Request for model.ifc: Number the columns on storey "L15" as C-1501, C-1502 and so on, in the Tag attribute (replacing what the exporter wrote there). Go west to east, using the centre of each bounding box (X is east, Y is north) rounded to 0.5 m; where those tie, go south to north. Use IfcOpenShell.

First a look at what the model holds.

```python
import ifcopenshell
import ifcopenshell.util.element
import ifcopenshell.util.placement

model = ifcopenshell.open("model.ifc")
print(model.schema)
storey = next(s for s in model.by_type("IfcBuildingStorey") if s.Name == "L15")
columns = [e for e in ifcopenshell.util.element.get_decomposition(storey) if e.is_a("IfcColumn")]
for e in sorted(columns, key=lambda e: e.id()):
    origin = ifcopenshell.util.placement.get_local_placement(e.ObjectPlacement)[:3, 3]
    print(e.id(), e.Tag, e.Name, origin.round(2) + 0.0, sep=" | ")
```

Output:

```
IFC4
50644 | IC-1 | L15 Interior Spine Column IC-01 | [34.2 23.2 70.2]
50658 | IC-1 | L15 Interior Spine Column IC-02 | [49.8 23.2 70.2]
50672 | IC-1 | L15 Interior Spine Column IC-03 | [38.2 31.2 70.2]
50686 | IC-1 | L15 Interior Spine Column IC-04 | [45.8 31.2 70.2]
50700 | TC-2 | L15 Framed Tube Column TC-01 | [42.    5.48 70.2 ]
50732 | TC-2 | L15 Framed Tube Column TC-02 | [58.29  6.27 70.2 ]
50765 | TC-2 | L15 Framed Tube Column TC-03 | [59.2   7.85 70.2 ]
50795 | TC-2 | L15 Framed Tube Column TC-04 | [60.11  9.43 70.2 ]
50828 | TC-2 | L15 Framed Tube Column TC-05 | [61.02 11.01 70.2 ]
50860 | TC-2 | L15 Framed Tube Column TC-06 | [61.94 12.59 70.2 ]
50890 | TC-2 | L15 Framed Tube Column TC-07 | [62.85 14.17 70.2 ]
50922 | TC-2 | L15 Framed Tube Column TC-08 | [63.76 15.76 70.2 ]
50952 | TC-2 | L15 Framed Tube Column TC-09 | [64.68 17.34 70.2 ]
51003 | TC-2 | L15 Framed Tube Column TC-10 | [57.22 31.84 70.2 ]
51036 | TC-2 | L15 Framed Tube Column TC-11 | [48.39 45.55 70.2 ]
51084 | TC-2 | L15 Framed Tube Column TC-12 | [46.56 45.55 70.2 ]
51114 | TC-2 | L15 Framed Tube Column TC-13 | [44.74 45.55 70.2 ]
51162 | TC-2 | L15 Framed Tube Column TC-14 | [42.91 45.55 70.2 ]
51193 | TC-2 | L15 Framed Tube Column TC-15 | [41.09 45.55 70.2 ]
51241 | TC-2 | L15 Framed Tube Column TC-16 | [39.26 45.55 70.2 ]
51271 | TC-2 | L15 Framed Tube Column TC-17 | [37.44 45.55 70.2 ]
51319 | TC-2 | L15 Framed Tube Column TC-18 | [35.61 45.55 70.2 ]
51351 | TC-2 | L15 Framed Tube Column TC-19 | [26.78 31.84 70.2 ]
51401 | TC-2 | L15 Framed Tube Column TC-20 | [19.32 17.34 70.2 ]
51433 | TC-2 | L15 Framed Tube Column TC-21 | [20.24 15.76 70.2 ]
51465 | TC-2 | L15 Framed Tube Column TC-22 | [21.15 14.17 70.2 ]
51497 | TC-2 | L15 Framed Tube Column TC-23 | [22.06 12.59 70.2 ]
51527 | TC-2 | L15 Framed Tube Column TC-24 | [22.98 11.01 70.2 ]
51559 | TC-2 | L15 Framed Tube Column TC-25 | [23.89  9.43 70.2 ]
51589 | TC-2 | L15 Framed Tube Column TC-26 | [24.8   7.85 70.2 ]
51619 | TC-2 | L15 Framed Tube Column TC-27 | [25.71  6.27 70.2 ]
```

```python
import ifcopenshell
import ifcopenshell.geom
import ifcopenshell.util.element
import ifcopenshell.util.shape

model = ifcopenshell.open("model.ifc")
settings = ifcopenshell.geom.settings()
settings.set("use-world-coords", True)


def centre(element):
    shape = ifcopenshell.geom.create_shape(settings, element)
    return ifcopenshell.util.shape.get_bbox_centroid(shape.geometry)


storey = next(s for s in model.by_type("IfcBuildingStorey") if s.Name == "L15")
columns = [e for e in ifcopenshell.util.element.get_decomposition(storey) if e.is_a("IfcColumn")]

# Insertion points can sit at a corner or the storey origin, so sort by the geometry (in metres).
centres = {e: centre(e) for e in columns}
columns.sort(key=lambda e: (round(centres[e][0] / 0.5), centres[e][1]))

for i, e in enumerate(columns, start=1):
    number = f"C-15{i:02d}"
    e.Tag = number
    print(e.id(), number)

model.write("model-out.ifc")
```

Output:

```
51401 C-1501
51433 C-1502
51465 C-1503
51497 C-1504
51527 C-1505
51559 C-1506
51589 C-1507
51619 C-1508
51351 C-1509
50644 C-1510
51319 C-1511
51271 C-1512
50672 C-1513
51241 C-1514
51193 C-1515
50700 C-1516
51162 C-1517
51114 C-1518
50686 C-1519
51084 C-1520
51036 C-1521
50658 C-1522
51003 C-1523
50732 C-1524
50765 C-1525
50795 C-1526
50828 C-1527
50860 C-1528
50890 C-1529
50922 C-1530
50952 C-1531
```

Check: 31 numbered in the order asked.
